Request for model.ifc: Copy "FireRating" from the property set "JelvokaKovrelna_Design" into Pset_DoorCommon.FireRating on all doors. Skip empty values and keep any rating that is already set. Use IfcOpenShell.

First a look at what the model holds.

```python
import ifcopenshell
import ifcopenshell.util.element

model = ifcopenshell.open("model.ifc")
print(model.schema)
doors = model.by_type("IfcDoor")
print(len(doors), "doors")
for e in doors[:8]:
    source = ifcopenshell.util.element.get_pset(e, "JelvokaKovrelna_Design", "FireRating")
    target = ifcopenshell.util.element.get_pset(e, "Pset_DoorCommon", "FireRating")
    print(e.id(), repr(source), repr(target), sep=" | ")
```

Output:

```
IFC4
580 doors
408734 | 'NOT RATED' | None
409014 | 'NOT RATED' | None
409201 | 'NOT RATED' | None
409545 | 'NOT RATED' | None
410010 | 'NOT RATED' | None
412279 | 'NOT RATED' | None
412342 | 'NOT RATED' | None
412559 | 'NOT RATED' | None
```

```python
import ifcopenshell
import ifcopenshell.api.pset
import ifcopenshell.util.element

model = ifcopenshell.open("model.ifc")

count = 0
for e in model.by_type("IfcDoor"):
    value = ifcopenshell.util.element.get_pset(e, "JelvokaKovrelna_Design", "FireRating")
    current = ifcopenshell.util.element.get_pset(e, "Pset_DoorCommon", "FireRating")
    if not value or not value.strip() or current:
        continue
    # add_pset returns the element's existing set when there is one.
    pset = ifcopenshell.api.pset.add_pset(model, product=e, name="Pset_DoorCommon")
    ifcopenshell.api.pset.edit_pset(model, pset=pset, properties={"FireRating": value})
    count += 1

print(count, "doors updated")

model.write("model_rev.ifc")
```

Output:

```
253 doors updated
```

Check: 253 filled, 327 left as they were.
